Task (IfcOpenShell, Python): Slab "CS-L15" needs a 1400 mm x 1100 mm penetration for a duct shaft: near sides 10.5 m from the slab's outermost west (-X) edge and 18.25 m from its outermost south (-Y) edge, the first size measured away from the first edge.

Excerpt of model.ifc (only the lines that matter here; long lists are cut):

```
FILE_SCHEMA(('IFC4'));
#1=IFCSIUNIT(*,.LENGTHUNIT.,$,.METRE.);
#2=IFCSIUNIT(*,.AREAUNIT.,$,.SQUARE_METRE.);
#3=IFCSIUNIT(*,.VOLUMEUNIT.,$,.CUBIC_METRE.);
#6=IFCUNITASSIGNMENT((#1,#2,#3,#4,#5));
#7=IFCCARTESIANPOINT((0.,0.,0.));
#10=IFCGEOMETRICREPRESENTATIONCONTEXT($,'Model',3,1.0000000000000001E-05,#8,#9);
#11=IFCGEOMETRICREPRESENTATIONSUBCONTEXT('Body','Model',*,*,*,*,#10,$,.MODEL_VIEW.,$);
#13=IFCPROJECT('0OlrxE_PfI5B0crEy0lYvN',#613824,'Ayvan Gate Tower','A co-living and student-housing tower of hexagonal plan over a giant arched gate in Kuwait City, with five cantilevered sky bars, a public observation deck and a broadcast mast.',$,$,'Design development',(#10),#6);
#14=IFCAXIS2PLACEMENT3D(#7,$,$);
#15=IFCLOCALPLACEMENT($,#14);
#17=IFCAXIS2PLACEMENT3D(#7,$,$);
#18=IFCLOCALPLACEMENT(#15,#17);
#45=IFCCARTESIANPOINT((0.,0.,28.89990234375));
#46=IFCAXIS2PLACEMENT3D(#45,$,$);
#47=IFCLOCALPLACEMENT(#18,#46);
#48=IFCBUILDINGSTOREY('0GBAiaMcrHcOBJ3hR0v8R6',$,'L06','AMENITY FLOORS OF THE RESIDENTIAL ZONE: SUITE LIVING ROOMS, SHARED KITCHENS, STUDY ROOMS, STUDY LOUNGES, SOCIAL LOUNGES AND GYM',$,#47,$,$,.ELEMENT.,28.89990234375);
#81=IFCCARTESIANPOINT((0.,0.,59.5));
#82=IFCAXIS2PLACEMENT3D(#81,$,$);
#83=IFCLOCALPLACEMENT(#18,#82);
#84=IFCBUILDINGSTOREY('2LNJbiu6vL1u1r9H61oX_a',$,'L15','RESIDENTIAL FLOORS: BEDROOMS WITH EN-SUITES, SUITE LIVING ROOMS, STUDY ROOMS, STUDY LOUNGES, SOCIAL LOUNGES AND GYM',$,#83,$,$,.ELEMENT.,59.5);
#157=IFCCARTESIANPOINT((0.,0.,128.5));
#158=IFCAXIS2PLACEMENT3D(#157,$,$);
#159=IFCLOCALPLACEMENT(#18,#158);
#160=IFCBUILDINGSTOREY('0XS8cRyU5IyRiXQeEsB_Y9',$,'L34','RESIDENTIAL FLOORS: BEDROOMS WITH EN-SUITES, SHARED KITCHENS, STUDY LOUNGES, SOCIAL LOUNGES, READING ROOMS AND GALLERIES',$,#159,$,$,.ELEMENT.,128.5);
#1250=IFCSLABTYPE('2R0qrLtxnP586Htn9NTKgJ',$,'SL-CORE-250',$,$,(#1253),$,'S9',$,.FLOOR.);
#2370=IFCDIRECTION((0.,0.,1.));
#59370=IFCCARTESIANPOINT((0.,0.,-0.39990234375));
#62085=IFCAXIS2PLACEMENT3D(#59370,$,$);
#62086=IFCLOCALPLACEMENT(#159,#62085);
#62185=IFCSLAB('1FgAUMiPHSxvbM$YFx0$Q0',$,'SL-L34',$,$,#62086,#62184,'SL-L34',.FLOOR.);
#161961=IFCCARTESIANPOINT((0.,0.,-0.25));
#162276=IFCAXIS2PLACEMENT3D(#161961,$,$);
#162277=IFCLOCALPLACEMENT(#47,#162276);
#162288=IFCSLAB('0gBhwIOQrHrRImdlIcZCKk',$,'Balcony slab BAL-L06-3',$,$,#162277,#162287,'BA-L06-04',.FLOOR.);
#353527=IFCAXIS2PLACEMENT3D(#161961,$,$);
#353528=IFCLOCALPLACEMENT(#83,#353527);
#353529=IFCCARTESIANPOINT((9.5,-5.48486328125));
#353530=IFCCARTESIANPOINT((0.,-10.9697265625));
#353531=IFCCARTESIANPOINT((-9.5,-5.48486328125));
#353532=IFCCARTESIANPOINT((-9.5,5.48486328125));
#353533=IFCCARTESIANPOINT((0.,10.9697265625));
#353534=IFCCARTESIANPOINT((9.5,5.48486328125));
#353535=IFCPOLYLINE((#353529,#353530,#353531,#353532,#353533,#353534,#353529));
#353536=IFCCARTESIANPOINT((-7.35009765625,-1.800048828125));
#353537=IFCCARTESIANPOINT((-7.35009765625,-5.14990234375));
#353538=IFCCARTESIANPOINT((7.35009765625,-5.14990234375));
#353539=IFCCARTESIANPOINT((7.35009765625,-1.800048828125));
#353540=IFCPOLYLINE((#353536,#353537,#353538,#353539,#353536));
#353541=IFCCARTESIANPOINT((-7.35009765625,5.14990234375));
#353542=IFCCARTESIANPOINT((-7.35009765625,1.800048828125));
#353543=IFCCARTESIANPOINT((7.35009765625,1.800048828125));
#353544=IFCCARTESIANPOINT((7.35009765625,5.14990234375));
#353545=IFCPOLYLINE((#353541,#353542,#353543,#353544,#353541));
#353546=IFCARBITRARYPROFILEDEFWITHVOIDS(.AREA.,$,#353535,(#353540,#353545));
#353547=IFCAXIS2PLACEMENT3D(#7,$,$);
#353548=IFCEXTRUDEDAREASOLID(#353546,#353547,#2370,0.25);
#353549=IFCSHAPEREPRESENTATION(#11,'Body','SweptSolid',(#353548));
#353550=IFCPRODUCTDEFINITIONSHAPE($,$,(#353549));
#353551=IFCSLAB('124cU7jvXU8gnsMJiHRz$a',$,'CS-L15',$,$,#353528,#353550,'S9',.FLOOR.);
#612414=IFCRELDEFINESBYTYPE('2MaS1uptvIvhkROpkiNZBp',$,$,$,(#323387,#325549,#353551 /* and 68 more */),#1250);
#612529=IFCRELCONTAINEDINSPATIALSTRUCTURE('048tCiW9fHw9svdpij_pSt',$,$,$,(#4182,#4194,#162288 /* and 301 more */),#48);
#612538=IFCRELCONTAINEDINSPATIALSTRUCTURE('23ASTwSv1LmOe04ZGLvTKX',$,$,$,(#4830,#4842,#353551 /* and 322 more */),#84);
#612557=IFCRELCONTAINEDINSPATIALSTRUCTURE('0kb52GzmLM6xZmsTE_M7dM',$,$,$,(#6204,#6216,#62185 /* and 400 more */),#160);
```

```python
import numpy as np
import ifcopenshell
import ifcopenshell.api.feature
import ifcopenshell.api.geometry
import ifcopenshell.api.root
import ifcopenshell.geom
import ifcopenshell.util.placement
import ifcopenshell.util.representation
import ifcopenshell.util.shape
import ifcopenshell.util.unit

model = ifcopenshell.open("model.ifc")
unit_scale = ifcopenshell.util.unit.calculate_unit_scale(model)
settings = ifcopenshell.geom.settings()


def volume(element):
    """Net volume in cubic metres, openings subtracted."""
    shape = ifcopenshell.geom.create_shape(settings, element)
    return ifcopenshell.util.shape.get_volume(shape.geometry)


slab = model.by_guid("124cU7jvXU8gnsMJiHRz$a")
before = volume(slab)

# Extent in the slab's own axes, in metres. The edges named are its -X and -Y sides.
slab_shape = ifcopenshell.geom.create_shape(settings, slab)
vertices = ifcopenshell.util.shape.get_vertices(slab_shape.geometry)
x_min, y_min, bottom = vertices.min(axis=0)
top = vertices[:, 2].max()

opening = ifcopenshell.api.root.create_entity(model, ifc_class="IfcOpeningElement", name="Duct shaft opening", predefined_type="OPENING")
context = ifcopenshell.util.representation.get_context(model, "Model", "Body", "MODEL_VIEW")
width, depth = 1.4, 1.1
outline = [(0.0, 0.0), (width, 0.0), (width, depth), (0.0, depth), (0.0, 0.0)]
# Overshoot both faces by 50 mm so the cut is clean.
shape = ifcopenshell.api.geometry.add_slab_representation(
    model, context=context, depth=top - bottom + 0.1, polyline=outline
)
ifcopenshell.api.geometry.assign_representation(model, product=opening, representation=shape)

matrix = ifcopenshell.util.placement.get_local_placement(slab.ObjectPlacement)
matrix[:, 3] = matrix @ np.append(np.array([x_min + 10.5, y_min + 18.25, bottom - 0.05]) / unit_scale, 1.0)
ifcopenshell.api.geometry.edit_object_placement(model, product=opening, matrix=matrix, is_si=False)
ifcopenshell.api.feature.add_feature(model, feature=opening, element=slab)

after = volume(slab)

print(f"slab volume {before:.3f} -> {after:.3f} m3")

model.write("model_v2.ifc")
```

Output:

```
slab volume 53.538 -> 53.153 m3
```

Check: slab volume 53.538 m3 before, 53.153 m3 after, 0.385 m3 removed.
